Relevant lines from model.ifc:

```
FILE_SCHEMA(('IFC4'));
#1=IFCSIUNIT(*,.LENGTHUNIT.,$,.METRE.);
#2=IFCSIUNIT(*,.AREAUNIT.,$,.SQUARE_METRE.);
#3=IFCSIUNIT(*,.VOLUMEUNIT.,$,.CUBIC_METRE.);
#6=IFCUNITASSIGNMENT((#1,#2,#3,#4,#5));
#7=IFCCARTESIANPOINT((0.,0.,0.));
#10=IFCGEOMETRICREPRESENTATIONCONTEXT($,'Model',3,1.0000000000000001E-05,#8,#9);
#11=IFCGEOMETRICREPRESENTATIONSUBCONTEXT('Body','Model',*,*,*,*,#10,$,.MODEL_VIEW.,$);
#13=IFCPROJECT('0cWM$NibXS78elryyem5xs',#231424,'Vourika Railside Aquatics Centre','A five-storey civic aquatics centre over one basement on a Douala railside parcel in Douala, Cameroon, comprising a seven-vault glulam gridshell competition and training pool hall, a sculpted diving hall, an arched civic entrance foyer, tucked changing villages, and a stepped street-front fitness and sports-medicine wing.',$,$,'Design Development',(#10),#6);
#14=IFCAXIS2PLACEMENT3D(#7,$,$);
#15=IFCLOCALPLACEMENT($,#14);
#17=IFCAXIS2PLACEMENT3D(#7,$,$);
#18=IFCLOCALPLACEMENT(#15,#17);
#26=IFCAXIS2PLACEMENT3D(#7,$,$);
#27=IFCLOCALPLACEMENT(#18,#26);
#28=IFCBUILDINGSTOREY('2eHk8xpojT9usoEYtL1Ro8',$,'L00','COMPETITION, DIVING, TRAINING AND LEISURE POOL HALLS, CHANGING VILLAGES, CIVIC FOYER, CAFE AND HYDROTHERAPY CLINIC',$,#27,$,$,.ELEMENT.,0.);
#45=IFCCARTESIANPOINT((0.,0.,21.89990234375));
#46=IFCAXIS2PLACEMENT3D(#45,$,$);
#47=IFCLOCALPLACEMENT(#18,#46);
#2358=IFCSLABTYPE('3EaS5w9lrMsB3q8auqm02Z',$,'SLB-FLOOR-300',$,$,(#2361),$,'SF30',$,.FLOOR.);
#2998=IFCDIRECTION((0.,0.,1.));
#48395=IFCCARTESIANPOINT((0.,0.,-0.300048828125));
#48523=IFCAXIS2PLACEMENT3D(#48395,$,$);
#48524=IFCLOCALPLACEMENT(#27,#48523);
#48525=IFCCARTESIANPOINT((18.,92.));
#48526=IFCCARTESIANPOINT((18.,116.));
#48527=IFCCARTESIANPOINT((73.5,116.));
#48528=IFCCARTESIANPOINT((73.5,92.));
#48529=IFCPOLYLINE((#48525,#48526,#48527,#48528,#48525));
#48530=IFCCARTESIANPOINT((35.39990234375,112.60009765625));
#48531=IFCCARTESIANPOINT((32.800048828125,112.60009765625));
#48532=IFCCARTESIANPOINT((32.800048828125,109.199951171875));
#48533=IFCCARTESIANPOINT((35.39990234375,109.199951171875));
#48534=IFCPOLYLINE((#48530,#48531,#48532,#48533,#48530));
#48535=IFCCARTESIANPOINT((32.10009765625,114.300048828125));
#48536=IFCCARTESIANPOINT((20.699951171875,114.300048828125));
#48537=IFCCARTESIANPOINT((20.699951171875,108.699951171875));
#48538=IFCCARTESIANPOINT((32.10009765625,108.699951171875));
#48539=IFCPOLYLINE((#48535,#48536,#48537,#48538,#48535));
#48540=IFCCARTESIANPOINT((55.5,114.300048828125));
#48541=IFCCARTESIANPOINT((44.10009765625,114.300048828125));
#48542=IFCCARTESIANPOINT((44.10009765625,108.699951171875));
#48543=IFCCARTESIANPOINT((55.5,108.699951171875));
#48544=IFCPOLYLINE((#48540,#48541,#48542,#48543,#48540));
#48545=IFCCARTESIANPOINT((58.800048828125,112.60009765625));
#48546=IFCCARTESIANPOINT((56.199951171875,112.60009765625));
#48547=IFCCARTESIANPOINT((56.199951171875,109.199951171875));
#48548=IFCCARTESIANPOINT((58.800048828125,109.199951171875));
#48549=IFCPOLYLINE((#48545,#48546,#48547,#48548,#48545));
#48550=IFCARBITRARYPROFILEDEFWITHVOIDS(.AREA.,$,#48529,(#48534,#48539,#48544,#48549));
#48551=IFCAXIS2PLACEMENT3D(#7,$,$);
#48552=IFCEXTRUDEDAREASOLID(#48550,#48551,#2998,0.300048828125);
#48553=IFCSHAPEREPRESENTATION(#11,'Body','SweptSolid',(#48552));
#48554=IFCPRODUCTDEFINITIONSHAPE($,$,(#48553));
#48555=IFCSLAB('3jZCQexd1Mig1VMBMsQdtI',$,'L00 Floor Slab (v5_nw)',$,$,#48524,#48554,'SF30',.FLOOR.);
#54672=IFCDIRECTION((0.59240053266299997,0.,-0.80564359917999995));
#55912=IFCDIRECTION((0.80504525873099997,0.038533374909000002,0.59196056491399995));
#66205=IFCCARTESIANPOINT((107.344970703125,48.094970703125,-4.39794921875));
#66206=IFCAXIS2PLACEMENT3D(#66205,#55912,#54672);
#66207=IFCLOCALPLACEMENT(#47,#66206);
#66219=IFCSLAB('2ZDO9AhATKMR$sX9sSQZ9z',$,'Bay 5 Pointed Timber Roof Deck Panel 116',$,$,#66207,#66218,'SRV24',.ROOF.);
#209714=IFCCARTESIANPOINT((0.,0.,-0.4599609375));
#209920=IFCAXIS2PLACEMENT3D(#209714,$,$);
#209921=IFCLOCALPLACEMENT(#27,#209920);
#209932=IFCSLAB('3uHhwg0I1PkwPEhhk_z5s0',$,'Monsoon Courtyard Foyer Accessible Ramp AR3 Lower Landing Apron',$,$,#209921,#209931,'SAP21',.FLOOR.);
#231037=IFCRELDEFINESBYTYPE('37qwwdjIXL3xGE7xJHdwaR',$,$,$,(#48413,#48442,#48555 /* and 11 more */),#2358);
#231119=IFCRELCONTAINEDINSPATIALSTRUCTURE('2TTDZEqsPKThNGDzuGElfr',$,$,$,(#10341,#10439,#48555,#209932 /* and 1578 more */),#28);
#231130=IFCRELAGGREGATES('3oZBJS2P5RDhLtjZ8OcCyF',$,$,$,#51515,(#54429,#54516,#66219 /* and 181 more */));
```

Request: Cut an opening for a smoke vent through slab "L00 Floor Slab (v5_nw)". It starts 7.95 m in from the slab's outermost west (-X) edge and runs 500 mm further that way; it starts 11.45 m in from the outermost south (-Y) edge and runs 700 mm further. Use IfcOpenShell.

```python
import numpy as np
import ifcopenshell
import ifcopenshell.api.feature
import ifcopenshell.api.geometry
import ifcopenshell.api.root
import ifcopenshell.geom
import ifcopenshell.util.placement
import ifcopenshell.util.representation
import ifcopenshell.util.shape
import ifcopenshell.util.unit

model = ifcopenshell.open("model.ifc")
unit_scale = ifcopenshell.util.unit.calculate_unit_scale(model)
settings = ifcopenshell.geom.settings()


def volume(element):
    """Net volume in cubic metres, openings subtracted."""
    shape = ifcopenshell.geom.create_shape(settings, element)
    return ifcopenshell.util.shape.get_volume(shape.geometry)


slab = model.by_guid("3jZCQexd1Mig1VMBMsQdtI")
before = volume(slab)

# Extent in the slab's own axes, in metres. The edges named are its -X and -Y sides.
slab_shape = ifcopenshell.geom.create_shape(settings, slab)
vertices = ifcopenshell.util.shape.get_vertices(slab_shape.geometry)
x_min, y_min, bottom = vertices.min(axis=0)
top = vertices[:, 2].max()

opening = ifcopenshell.api.root.create_entity(model, ifc_class="IfcOpeningElement", name="Smoke vent opening", predefined_type="OPENING")
context = ifcopenshell.util.representation.get_context(model, "Model", "Body", "MODEL_VIEW")
width, depth = 0.5, 0.7
outline = [(0.0, 0.0), (width, 0.0), (width, depth), (0.0, depth), (0.0, 0.0)]
# Overshoot both faces by 50 mm so the cut is clean.
shape = ifcopenshell.api.geometry.add_slab_representation(
    model, context=context, depth=top - bottom + 0.1, polyline=outline
)
ifcopenshell.api.geometry.assign_representation(model, product=opening, representation=shape)

matrix = ifcopenshell.util.placement.get_local_placement(slab.ObjectPlacement)
matrix[:, 3] = matrix @ np.append(np.array([x_min + 7.95, y_min + 11.45, bottom - 0.05]) / unit_scale, 1.0)
ifcopenshell.api.geometry.edit_object_placement(model, product=opening, matrix=matrix, is_si=False)
ifcopenshell.api.feature.add_feature(model, feature=opening, element=slab)

after = volume(slab)

print(f"slab volume {before:.3f} -> {after:.3f} m3")

model.write("model_rev.ifc")
```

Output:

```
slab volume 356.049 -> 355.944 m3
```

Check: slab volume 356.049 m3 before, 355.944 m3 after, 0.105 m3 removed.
